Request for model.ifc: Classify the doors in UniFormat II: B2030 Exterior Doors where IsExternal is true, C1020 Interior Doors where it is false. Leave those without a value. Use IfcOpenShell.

First a look at what the model holds.

```python
import ifcopenshell
import ifcopenshell.util.element

model = ifcopenshell.open("model.ifc")
print(model.schema)
print("classifications:", [c.Name for c in model.by_type("IfcClassification")])
values = [ifcopenshell.util.element.get_pset(e, "Pset_DoorCommon", "IsExternal") for e in model.by_type("IfcDoor")]
for value in (True, False, None):
    print("IsExternal", value, values.count(value))
```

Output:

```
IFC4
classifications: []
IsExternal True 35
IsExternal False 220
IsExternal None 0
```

```python
import ifcopenshell
import ifcopenshell.api.classification
import ifcopenshell.util.element

model = ifcopenshell.open("model.ifc")

system = ifcopenshell.api.classification.add_classification(model, classification="UniFormat II")

doors = model.by_type("IfcDoor")
external = {e: ifcopenshell.util.element.get_pset(e, "Pset_DoorCommon", "IsExternal") for e in doors}
for flag, code, name in ((True, "B2030", "Exterior Doors"), (False, "C1020", "Interior Doors")):
    products = [e for e in doors if external[e] is flag]
    ifcopenshell.api.classification.add_reference(
        model, products=products, classification=system, identification=code, name=name
    )
    print(code, len(products))

model.write("model_edited.ifc")
```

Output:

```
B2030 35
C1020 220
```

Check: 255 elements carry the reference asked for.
